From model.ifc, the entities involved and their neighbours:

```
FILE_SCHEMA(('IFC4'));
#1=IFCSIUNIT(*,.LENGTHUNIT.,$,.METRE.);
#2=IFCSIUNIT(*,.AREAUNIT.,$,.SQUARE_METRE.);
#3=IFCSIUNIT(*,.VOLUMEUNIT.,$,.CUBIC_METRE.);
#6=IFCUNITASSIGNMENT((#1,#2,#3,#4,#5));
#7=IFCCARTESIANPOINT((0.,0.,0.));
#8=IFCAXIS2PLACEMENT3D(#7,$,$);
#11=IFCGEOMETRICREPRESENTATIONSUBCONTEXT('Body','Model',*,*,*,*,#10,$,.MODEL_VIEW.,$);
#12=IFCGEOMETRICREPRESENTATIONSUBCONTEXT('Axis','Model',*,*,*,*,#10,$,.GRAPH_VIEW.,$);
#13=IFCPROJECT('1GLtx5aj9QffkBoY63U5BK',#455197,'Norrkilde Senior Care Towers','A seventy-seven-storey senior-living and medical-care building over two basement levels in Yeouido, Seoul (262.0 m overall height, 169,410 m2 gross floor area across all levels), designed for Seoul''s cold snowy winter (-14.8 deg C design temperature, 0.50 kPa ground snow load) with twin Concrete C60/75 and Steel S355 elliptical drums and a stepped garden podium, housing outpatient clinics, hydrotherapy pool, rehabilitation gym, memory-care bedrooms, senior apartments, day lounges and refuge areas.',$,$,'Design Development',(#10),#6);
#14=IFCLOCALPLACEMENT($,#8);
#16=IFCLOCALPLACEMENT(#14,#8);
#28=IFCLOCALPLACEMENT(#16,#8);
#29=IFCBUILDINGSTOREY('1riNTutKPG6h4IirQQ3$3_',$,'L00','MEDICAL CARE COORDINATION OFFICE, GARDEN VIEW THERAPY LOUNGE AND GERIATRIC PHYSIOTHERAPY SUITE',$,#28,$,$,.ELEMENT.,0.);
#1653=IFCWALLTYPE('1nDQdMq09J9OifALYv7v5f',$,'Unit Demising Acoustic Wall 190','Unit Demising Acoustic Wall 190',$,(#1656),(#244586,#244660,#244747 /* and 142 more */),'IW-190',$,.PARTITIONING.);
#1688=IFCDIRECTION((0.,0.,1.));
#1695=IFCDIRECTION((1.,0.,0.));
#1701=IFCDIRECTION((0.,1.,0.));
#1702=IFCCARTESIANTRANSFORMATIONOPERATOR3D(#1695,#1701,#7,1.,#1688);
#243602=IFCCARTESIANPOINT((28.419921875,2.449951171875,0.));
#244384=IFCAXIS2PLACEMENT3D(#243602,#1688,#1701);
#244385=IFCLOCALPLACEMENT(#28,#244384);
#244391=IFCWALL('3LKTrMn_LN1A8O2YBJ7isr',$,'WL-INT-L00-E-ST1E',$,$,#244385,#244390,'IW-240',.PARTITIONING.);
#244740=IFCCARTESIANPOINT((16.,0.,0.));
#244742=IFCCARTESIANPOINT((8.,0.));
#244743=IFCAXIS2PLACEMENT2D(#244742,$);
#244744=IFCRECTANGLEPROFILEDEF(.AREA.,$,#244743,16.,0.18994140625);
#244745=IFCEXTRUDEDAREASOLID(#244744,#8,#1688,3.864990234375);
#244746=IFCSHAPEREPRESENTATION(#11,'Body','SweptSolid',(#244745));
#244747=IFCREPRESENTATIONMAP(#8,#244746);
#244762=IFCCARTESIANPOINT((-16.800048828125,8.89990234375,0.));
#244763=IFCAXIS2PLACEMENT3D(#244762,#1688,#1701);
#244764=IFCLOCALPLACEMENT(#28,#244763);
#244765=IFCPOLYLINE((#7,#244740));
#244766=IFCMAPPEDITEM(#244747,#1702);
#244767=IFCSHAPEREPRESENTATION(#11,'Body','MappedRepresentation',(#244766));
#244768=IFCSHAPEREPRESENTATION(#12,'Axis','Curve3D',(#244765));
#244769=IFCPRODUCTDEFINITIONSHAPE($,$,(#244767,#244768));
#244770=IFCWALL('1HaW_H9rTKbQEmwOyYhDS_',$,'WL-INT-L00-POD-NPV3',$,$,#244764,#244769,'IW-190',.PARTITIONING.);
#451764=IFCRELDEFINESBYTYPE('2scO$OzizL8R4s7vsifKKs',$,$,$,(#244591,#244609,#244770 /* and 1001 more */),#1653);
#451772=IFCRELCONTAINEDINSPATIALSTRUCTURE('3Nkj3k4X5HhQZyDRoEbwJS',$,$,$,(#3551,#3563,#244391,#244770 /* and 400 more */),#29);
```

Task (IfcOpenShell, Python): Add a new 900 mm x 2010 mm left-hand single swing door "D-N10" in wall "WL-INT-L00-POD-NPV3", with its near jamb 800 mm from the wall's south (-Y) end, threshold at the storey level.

```python
import numpy as np
import ifcopenshell
import ifcopenshell.api.feature
import ifcopenshell.api.geometry
import ifcopenshell.api.root
import ifcopenshell.api.spatial
import ifcopenshell.geom
import ifcopenshell.util.element
import ifcopenshell.util.placement
import ifcopenshell.util.representation
import ifcopenshell.util.shape
import ifcopenshell.util.unit

model = ifcopenshell.open("model.ifc")
unit_scale = ifcopenshell.util.unit.calculate_unit_scale(model)
settings = ifcopenshell.geom.settings()


def volume(element):
    """Net volume in cubic metres, openings subtracted."""
    shape = ifcopenshell.geom.create_shape(settings, element)
    return ifcopenshell.util.shape.get_volume(shape.geometry)


wall = model.by_guid("1HaW_H9rTKbQEmwOyYhDS_")
storey = ifcopenshell.util.element.get_container(wall, ifc_class="IfcBuildingStorey")
context = ifcopenshell.util.representation.get_context(model, "Model", "Body", "MODEL_VIEW")
before = volume(wall)

width, height, from_end, sill = 0.9, 2.01, 0.8, 0.0  # metres

# The wall runs along its own X axis, and the end named is its -X end.
wall_shape = ifcopenshell.geom.create_shape(settings, wall)
x, y, z = ifcopenshell.util.shape.get_vertices(wall_shape.geometry).T
start = x.min() + from_end
face, thickness = float(y.min()), float(y.max() - y.min())
wall_matrix = ifcopenshell.util.placement.get_local_placement(wall.ObjectPlacement)
level = ifcopenshell.util.placement.get_local_placement(storey.ObjectPlacement)[2, 3]


def in_wall(x, y):
    """Placement at x, y metres in the wall's axes, at sill height."""
    matrix = wall_matrix.copy()
    matrix[:, 3] = wall_matrix @ np.array([x / unit_scale, y / unit_scale, 0.0, 1.0])
    matrix[2, 3] = level + sill / unit_scale
    return matrix


# Opening: a box that overshoots both wall faces by 50 mm.
opening = ifcopenshell.api.root.create_entity(model, ifc_class="IfcOpeningElement", predefined_type="OPENING")
box = ifcopenshell.api.geometry.add_wall_representation(
    model, context=context, length=width, height=height, thickness=thickness + 0.1
)
ifcopenshell.api.geometry.assign_representation(model, product=opening, representation=box)
ifcopenshell.api.geometry.edit_object_placement(model, product=opening, matrix=in_wall(start, face - 0.05), is_si=False)
ifcopenshell.api.feature.add_feature(model, feature=opening, element=wall)

door = ifcopenshell.api.root.create_entity(model, ifc_class="IfcDoor", name="D-N10", predefined_type="DOOR")
door.OverallWidth, door.OverallHeight = width / unit_scale, height / unit_scale
door.OperationType = "SINGLE_SWING_LEFT"
body = ifcopenshell.api.geometry.add_door_representation(
    model,
    context=context,
    overall_width=door.OverallWidth,
    overall_height=door.OverallHeight,
    operation_type="SINGLE_SWING_LEFT",
    lining_properties={"LiningDepth": thickness / unit_scale, "ThresholdDepth": thickness / unit_scale},
)
ifcopenshell.api.geometry.assign_representation(model, product=door, representation=body)
ifcopenshell.api.spatial.assign_container(model, products=[door], relating_structure=storey)
ifcopenshell.api.feature.add_filling(model, opening=opening, element=door)

# The lining spans the wall, so the door starts at the wall face.
ifcopenshell.api.geometry.edit_object_placement(model, product=door, matrix=in_wall(start, face), is_si=False)

after = volume(wall)

print(f"wall volume {before:.3f} -> {after:.3f} m3")

model.write("model_updated.ifc")
```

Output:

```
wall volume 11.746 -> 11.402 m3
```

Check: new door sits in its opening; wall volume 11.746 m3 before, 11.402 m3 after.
